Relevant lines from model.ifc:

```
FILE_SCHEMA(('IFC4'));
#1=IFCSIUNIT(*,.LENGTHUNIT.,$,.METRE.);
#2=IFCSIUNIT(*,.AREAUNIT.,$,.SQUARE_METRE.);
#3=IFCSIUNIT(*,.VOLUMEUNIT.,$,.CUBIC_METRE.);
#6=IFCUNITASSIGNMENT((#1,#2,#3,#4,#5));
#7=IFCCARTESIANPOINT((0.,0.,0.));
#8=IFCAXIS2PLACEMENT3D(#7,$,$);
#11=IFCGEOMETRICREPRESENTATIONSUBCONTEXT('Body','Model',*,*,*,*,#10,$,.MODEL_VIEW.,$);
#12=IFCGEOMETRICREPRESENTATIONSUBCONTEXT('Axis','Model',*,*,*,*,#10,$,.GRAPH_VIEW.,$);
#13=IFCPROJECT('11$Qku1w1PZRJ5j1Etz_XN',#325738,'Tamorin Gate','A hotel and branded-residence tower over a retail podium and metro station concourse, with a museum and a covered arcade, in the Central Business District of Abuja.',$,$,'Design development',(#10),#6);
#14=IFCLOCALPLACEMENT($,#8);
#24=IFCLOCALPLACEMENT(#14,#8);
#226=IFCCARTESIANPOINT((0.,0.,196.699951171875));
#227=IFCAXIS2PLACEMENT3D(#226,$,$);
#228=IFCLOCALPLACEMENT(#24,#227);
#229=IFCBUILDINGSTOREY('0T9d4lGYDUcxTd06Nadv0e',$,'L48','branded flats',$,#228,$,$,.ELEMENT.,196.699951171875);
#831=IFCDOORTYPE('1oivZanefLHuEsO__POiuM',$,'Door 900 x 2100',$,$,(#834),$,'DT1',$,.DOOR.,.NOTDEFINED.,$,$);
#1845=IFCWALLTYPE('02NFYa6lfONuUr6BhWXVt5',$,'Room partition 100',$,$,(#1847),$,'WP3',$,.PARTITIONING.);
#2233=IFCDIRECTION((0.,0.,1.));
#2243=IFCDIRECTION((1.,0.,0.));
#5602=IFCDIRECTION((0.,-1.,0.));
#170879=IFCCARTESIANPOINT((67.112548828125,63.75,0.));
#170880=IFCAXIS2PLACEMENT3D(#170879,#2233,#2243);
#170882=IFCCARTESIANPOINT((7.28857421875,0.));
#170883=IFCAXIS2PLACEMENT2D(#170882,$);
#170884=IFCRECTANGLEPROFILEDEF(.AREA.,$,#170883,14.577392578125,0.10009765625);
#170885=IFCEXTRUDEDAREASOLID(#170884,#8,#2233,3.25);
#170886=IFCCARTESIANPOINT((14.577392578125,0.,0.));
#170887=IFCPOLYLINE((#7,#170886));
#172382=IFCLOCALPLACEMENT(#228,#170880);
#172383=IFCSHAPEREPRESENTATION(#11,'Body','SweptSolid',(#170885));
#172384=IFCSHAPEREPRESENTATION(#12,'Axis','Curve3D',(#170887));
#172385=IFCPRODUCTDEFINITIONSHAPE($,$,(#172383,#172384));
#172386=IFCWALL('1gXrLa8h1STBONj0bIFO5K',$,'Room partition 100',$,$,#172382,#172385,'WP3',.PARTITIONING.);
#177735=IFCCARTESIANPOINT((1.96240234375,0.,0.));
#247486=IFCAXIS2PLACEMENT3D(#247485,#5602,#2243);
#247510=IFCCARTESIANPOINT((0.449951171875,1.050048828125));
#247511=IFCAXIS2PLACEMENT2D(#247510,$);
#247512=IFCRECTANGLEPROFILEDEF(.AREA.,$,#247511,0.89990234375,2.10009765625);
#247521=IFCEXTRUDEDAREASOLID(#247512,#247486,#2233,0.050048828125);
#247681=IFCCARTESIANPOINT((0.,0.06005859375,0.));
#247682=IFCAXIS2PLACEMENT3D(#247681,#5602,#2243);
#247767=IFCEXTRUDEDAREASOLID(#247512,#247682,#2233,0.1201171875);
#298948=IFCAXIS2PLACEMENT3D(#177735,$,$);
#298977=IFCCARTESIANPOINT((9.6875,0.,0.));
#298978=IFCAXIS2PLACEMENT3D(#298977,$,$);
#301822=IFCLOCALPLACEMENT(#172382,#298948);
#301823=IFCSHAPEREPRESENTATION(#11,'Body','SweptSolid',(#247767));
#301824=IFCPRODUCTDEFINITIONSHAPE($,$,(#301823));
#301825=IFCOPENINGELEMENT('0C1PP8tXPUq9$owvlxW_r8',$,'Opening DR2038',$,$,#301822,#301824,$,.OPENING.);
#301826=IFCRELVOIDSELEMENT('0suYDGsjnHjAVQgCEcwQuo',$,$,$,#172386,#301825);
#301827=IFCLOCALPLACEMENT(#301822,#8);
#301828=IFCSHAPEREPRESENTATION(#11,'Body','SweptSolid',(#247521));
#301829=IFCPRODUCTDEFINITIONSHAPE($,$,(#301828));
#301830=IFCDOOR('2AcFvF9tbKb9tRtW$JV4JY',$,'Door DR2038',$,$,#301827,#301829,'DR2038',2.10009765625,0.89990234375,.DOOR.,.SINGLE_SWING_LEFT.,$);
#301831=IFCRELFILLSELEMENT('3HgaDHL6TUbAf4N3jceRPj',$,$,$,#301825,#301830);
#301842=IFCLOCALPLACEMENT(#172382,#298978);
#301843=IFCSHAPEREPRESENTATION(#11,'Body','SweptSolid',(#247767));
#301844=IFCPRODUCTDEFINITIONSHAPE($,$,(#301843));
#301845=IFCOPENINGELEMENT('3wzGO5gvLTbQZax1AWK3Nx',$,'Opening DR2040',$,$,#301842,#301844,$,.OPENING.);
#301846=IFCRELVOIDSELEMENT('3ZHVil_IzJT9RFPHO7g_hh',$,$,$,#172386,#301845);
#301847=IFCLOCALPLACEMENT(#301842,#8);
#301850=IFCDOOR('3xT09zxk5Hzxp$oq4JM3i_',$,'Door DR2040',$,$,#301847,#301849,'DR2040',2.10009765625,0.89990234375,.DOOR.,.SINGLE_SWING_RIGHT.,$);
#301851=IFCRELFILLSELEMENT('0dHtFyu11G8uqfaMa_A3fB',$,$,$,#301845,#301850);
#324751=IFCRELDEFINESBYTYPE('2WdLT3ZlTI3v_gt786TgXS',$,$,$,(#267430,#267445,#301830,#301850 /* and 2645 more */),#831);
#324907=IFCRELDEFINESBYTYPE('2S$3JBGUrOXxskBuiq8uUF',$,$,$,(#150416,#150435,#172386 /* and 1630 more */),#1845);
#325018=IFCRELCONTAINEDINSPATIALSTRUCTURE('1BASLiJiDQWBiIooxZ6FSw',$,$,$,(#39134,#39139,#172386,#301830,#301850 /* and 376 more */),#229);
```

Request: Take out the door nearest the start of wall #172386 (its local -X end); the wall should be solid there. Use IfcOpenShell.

```python
import ifcopenshell
import ifcopenshell.api.feature
import ifcopenshell.api.root
import ifcopenshell.geom
import ifcopenshell.util.shape

model = ifcopenshell.open("model.ifc")
settings = ifcopenshell.geom.settings()


def volume(element):
    """Net volume in cubic metres, openings subtracted."""
    shape = ifcopenshell.geom.create_shape(settings, element)
    return ifcopenshell.util.shape.get_volume(shape.geometry)


door = model.by_id(301830)
opening = door.FillsVoids[0].RelatingOpeningElement
wall = opening.VoidsElements[0].RelatingBuildingElement
before = volume(wall)

ifcopenshell.api.root.remove_product(model, product=door)
ifcopenshell.api.feature.remove_feature(model, feature=opening)

after = volume(wall)

print(f"wall volume {before:.3f} -> {after:.3f} m3")

model.write("model_rev.ifc")
```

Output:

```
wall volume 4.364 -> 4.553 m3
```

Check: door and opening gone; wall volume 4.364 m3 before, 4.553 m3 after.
